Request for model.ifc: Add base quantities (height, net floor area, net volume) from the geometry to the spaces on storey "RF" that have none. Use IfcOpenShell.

First a look at what the model holds.

```python
import ifcopenshell
import ifcopenshell.util.element
import ifcopenshell.util.unit

model = ifcopenshell.open("model.ifc")
print(model.schema)
for unit_type in ("LENGTHUNIT", "AREAUNIT", "VOLUMEUNIT"):
    print(unit_type, ifcopenshell.util.unit.calculate_unit_scale(model, unit_type))
storey = next(s for s in model.by_type("IfcBuildingStorey") if s.Name == "RF")
spaces = [e for e in ifcopenshell.util.element.get_decomposition(storey) if e.is_a("IfcSpace")]
for e in sorted(spaces, key=lambda e: e.id()):
    print(e.id(), e.is_a(), e.Name, list(ifcopenshell.util.element.get_psets(e, qtos_only=True)), sep=" | ")
```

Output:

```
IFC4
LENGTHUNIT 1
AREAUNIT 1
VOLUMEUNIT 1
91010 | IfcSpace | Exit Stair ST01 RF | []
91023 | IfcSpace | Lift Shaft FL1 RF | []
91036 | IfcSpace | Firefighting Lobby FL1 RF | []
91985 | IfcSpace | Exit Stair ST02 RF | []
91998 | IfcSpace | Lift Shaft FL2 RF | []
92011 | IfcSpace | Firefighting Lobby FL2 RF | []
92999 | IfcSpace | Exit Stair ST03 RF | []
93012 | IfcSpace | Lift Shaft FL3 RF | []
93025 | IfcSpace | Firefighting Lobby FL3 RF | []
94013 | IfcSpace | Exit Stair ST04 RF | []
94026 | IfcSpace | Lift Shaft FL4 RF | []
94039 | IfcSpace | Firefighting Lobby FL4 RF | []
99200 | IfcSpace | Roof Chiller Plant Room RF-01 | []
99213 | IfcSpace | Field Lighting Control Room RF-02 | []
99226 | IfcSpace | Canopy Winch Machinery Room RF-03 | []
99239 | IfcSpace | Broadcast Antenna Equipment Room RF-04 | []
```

```python
import ifcopenshell
import ifcopenshell.api.pset
import ifcopenshell.geom
import ifcopenshell.util.element
import ifcopenshell.util.shape
import ifcopenshell.util.unit

model = ifcopenshell.open("model.ifc")
unit_scale = ifcopenshell.util.unit.calculate_unit_scale(model)
area_scale = ifcopenshell.util.unit.calculate_unit_scale(model, "AREAUNIT")
volume_scale = ifcopenshell.util.unit.calculate_unit_scale(model, "VOLUMEUNIT")
settings = ifcopenshell.geom.settings()

storey = next(s for s in model.by_type("IfcBuildingStorey") if s.Name == "RF")
spaces = [e for e in ifcopenshell.util.element.get_decomposition(storey) if e.is_a("IfcSpace")]

for e in sorted(spaces, key=lambda e: e.id()):
    if ifcopenshell.util.element.get_psets(e, qtos_only=True, should_inherit=False):
        continue
    # Geometry comes back in metres, in the element's own axes.
    shape = ifcopenshell.geom.create_shape(settings, e)
    values = {
        "Height": ifcopenshell.util.shape.get_z(shape.geometry) / unit_scale,
        "NetFloorArea": ifcopenshell.util.shape.get_footprint_area(shape.geometry) / area_scale,
        "NetVolume": ifcopenshell.util.shape.get_volume(shape.geometry) / volume_scale,
    }
    qto = ifcopenshell.api.pset.add_qto(model, product=e, name="Qto_SpaceBaseQuantities")
    ifcopenshell.api.pset.edit_qto(model, qto=qto, properties=values)
    print(e.id(), {k: round(v, 3) for k, v in values.items()})

model.write("model_rev.ifc")
```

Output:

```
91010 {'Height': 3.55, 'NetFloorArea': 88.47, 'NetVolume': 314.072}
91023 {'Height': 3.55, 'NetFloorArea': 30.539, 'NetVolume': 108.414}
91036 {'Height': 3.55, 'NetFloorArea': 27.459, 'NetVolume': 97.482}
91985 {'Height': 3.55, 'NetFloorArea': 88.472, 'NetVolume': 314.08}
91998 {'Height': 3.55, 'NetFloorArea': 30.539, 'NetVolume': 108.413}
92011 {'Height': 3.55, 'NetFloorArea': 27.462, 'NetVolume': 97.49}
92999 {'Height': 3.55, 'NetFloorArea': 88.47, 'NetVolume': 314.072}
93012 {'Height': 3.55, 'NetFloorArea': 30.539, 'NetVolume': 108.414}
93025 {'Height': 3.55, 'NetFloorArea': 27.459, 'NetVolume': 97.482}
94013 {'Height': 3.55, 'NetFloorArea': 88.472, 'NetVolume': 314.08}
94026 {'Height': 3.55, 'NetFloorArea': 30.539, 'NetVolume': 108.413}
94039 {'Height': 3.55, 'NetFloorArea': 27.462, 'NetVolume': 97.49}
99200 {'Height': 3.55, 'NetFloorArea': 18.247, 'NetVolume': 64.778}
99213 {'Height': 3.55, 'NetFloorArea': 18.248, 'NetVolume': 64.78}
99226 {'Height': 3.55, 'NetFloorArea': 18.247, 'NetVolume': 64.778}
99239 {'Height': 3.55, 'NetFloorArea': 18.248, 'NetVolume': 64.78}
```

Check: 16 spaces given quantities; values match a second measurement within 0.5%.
